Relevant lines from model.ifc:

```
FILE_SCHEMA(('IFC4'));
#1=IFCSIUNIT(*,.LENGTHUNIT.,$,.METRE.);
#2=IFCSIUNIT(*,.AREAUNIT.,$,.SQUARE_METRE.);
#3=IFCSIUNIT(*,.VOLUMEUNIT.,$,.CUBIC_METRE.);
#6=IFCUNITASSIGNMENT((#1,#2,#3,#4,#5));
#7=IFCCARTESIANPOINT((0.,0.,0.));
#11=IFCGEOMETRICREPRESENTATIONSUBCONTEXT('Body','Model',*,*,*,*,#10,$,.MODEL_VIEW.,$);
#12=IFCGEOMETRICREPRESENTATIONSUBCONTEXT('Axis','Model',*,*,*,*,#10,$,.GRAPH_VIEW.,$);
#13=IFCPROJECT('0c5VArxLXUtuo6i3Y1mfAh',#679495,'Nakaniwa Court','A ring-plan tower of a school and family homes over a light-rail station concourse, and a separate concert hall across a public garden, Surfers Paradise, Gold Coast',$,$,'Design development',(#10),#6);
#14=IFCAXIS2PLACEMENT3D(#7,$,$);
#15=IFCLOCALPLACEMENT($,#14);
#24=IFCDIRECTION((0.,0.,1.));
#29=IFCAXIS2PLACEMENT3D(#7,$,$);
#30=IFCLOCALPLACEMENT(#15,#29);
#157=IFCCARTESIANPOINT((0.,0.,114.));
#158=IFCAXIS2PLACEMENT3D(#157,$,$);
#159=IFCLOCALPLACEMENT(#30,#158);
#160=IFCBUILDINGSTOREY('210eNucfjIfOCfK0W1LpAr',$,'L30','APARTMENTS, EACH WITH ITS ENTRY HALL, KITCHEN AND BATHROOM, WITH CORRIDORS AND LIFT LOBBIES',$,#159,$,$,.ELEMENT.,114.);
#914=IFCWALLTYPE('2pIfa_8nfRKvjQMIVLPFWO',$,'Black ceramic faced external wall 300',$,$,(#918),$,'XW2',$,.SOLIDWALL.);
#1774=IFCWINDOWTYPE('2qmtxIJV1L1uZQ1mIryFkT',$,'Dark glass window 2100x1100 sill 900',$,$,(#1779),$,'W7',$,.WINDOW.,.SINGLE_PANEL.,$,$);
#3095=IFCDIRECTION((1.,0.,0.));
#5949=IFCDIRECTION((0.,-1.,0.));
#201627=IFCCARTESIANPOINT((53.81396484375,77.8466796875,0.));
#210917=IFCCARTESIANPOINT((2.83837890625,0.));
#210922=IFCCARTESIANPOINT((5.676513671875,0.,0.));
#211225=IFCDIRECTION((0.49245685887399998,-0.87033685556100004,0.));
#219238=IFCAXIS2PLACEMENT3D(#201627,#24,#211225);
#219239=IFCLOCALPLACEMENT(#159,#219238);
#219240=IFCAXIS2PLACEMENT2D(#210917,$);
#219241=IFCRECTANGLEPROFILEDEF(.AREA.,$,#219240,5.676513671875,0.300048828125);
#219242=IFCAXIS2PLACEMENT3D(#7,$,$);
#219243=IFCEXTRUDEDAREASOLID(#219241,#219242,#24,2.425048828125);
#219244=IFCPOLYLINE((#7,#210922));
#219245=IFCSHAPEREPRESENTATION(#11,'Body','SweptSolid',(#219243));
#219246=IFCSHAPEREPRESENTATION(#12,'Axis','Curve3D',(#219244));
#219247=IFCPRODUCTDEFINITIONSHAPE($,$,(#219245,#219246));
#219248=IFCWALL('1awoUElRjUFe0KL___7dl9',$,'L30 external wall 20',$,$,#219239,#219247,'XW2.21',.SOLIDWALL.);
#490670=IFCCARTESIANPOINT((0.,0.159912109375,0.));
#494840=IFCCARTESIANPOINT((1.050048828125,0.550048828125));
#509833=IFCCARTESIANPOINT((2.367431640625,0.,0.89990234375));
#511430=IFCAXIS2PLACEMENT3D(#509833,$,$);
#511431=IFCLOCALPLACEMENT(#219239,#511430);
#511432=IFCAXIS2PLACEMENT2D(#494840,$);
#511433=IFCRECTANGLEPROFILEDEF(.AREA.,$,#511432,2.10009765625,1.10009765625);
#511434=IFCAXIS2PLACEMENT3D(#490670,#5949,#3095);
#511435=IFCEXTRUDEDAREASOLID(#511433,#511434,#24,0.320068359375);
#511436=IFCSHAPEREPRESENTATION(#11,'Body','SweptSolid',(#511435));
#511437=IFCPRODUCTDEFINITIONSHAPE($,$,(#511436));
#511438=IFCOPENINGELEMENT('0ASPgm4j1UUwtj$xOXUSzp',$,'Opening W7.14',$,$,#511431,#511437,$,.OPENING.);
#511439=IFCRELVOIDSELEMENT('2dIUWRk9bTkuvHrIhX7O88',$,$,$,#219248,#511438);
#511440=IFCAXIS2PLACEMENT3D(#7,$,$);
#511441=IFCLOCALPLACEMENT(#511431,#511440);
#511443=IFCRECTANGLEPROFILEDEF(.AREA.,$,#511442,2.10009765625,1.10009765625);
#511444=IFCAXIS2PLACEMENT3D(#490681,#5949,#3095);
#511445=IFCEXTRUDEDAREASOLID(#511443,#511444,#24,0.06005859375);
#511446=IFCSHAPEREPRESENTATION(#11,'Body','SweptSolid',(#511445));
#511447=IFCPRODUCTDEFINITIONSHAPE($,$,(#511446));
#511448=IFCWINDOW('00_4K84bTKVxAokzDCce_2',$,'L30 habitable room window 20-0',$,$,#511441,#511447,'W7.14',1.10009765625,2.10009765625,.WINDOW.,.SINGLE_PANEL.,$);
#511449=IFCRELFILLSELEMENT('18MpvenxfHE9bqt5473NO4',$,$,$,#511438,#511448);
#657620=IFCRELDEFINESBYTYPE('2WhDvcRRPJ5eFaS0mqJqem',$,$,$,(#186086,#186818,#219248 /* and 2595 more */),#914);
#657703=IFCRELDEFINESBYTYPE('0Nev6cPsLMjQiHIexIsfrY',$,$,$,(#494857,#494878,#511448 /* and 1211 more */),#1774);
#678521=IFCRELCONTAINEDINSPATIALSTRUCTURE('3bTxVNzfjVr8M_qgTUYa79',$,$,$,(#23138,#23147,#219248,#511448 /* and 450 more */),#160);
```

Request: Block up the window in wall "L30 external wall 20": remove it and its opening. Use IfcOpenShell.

```python
import ifcopenshell
import ifcopenshell.api.feature
import ifcopenshell.api.root
import ifcopenshell.geom
import ifcopenshell.util.shape

model = ifcopenshell.open("model.ifc")
settings = ifcopenshell.geom.settings()


def volume(element):
    """Net volume in cubic metres, openings subtracted."""
    shape = ifcopenshell.geom.create_shape(settings, element)
    return ifcopenshell.util.shape.get_volume(shape.geometry)


window = model.by_guid("00_4K84bTKVxAokzDCce_2")
opening = window.FillsVoids[0].RelatingOpeningElement
wall = opening.VoidsElements[0].RelatingBuildingElement
before = volume(wall)

ifcopenshell.api.root.remove_product(model, product=window)
ifcopenshell.api.feature.remove_feature(model, feature=opening)

after = volume(wall)

print(f"wall volume {before:.3f} -> {after:.3f} m3")

model.write("model_rev.ifc")
```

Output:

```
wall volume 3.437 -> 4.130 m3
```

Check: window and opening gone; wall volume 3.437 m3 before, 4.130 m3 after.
